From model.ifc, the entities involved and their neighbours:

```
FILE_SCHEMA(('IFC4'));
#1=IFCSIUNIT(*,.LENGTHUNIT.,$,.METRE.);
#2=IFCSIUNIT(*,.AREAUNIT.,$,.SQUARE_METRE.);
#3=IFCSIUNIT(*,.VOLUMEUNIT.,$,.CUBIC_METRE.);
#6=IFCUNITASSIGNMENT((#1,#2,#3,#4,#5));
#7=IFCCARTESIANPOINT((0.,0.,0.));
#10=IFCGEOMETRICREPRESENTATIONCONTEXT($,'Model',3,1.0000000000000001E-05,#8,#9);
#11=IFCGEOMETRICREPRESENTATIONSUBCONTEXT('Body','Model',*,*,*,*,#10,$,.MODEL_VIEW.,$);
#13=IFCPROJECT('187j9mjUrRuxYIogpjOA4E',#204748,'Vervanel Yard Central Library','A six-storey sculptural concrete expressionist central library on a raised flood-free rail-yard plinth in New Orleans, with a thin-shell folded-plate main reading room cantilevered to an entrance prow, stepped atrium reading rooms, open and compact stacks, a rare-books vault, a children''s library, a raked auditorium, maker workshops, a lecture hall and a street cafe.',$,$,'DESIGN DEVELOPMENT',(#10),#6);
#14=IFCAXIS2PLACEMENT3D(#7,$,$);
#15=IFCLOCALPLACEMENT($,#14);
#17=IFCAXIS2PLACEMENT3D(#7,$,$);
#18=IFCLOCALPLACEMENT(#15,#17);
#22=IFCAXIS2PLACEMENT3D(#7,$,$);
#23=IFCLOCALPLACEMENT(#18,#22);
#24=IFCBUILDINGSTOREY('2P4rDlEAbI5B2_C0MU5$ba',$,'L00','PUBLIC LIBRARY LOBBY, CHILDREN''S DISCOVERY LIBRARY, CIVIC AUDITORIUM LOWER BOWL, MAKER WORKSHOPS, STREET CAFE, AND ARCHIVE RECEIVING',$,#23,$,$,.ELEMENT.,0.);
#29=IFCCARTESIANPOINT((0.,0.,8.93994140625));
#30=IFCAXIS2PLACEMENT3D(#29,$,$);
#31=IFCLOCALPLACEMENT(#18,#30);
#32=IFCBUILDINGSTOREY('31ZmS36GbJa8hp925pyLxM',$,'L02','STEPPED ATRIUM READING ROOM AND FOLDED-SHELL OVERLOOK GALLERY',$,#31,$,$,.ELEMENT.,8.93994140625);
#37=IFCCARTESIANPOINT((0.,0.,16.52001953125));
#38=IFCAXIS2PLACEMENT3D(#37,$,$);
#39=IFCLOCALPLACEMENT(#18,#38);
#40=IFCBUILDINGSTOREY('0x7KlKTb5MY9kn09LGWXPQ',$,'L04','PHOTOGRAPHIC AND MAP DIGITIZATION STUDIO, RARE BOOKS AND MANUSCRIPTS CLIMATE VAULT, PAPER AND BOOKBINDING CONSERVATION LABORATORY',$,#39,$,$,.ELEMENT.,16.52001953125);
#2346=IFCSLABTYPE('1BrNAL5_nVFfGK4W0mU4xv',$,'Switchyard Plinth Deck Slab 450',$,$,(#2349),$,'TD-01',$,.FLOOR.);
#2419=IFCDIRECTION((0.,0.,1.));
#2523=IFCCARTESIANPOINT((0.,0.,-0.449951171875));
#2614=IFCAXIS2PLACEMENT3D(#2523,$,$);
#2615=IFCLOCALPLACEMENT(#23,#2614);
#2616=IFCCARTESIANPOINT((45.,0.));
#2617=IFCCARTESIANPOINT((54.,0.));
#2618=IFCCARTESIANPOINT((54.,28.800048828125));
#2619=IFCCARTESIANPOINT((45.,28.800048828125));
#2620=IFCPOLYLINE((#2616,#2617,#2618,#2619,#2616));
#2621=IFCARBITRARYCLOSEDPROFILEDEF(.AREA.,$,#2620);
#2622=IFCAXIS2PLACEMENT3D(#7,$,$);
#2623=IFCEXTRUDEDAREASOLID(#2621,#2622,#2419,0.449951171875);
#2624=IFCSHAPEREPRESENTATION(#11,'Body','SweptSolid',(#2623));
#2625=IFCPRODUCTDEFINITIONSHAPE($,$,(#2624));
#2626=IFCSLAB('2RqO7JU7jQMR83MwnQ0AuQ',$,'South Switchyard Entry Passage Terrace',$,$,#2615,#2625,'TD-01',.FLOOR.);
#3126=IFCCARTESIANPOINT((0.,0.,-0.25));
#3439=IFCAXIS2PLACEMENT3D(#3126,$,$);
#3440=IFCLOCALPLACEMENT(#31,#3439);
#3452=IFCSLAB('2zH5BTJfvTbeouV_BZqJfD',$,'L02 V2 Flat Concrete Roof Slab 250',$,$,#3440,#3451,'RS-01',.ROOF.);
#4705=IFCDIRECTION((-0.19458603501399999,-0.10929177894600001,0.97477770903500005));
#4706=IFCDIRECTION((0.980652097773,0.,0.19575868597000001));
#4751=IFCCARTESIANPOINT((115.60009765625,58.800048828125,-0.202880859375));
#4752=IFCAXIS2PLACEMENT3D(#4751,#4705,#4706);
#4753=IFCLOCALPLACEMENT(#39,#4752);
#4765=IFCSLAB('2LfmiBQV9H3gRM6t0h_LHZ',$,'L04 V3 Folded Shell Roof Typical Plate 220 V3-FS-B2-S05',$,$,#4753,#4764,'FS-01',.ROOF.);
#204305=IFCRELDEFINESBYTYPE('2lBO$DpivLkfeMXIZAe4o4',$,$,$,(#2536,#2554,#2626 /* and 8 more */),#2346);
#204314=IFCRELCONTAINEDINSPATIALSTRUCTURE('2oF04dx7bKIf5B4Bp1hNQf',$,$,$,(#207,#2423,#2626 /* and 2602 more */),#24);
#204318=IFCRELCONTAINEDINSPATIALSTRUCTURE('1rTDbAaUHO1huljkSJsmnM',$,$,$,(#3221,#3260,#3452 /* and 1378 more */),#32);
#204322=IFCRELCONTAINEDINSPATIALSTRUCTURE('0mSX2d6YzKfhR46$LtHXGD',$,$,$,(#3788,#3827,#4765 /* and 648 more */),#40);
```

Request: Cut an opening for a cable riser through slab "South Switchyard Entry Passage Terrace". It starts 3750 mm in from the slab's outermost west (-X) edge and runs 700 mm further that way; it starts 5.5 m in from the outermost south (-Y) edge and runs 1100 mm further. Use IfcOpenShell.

```python
import numpy as np
import ifcopenshell
import ifcopenshell.api.feature
import ifcopenshell.api.geometry
import ifcopenshell.api.root
import ifcopenshell.geom
import ifcopenshell.util.placement
import ifcopenshell.util.representation
import ifcopenshell.util.shape
import ifcopenshell.util.unit

model = ifcopenshell.open("model.ifc")
unit_scale = ifcopenshell.util.unit.calculate_unit_scale(model)
settings = ifcopenshell.geom.settings()


def volume(element):
    """Net volume in cubic metres, openings subtracted."""
    shape = ifcopenshell.geom.create_shape(settings, element)
    return ifcopenshell.util.shape.get_volume(shape.geometry)


slab = model.by_guid("2RqO7JU7jQMR83MwnQ0AuQ")
before = volume(slab)

# Extent in the slab's own axes, in metres. The edges named are its -X and -Y sides.
slab_shape = ifcopenshell.geom.create_shape(settings, slab)
vertices = ifcopenshell.util.shape.get_vertices(slab_shape.geometry)
x_min, y_min, bottom = vertices.min(axis=0)
top = vertices[:, 2].max()

opening = ifcopenshell.api.root.create_entity(model, ifc_class="IfcOpeningElement", name="Cable riser opening", predefined_type="OPENING")
context = ifcopenshell.util.representation.get_context(model, "Model", "Body", "MODEL_VIEW")
width, depth = 0.7, 1.1
outline = [(0.0, 0.0), (width, 0.0), (width, depth), (0.0, depth), (0.0, 0.0)]
# Overshoot both faces by 50 mm so the cut is clean.
shape = ifcopenshell.api.geometry.add_slab_representation(
    model, context=context, depth=top - bottom + 0.1, polyline=outline
)
ifcopenshell.api.geometry.assign_representation(model, product=opening, representation=shape)

matrix = ifcopenshell.util.placement.get_local_placement(slab.ObjectPlacement)
matrix[:, 3] = matrix @ np.append(np.array([x_min + 3.75, y_min + 5.5, bottom - 0.05]) / unit_scale, 1.0)
ifcopenshell.api.geometry.edit_object_placement(model, product=opening, matrix=matrix, is_si=False)
ifcopenshell.api.feature.add_feature(model, feature=opening, element=slab)

after = volume(slab)

print(f"slab volume {before:.3f} -> {after:.3f} m3")

model.write("model_rev.ifc")
```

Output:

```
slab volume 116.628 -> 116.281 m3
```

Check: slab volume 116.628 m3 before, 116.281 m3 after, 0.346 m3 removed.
